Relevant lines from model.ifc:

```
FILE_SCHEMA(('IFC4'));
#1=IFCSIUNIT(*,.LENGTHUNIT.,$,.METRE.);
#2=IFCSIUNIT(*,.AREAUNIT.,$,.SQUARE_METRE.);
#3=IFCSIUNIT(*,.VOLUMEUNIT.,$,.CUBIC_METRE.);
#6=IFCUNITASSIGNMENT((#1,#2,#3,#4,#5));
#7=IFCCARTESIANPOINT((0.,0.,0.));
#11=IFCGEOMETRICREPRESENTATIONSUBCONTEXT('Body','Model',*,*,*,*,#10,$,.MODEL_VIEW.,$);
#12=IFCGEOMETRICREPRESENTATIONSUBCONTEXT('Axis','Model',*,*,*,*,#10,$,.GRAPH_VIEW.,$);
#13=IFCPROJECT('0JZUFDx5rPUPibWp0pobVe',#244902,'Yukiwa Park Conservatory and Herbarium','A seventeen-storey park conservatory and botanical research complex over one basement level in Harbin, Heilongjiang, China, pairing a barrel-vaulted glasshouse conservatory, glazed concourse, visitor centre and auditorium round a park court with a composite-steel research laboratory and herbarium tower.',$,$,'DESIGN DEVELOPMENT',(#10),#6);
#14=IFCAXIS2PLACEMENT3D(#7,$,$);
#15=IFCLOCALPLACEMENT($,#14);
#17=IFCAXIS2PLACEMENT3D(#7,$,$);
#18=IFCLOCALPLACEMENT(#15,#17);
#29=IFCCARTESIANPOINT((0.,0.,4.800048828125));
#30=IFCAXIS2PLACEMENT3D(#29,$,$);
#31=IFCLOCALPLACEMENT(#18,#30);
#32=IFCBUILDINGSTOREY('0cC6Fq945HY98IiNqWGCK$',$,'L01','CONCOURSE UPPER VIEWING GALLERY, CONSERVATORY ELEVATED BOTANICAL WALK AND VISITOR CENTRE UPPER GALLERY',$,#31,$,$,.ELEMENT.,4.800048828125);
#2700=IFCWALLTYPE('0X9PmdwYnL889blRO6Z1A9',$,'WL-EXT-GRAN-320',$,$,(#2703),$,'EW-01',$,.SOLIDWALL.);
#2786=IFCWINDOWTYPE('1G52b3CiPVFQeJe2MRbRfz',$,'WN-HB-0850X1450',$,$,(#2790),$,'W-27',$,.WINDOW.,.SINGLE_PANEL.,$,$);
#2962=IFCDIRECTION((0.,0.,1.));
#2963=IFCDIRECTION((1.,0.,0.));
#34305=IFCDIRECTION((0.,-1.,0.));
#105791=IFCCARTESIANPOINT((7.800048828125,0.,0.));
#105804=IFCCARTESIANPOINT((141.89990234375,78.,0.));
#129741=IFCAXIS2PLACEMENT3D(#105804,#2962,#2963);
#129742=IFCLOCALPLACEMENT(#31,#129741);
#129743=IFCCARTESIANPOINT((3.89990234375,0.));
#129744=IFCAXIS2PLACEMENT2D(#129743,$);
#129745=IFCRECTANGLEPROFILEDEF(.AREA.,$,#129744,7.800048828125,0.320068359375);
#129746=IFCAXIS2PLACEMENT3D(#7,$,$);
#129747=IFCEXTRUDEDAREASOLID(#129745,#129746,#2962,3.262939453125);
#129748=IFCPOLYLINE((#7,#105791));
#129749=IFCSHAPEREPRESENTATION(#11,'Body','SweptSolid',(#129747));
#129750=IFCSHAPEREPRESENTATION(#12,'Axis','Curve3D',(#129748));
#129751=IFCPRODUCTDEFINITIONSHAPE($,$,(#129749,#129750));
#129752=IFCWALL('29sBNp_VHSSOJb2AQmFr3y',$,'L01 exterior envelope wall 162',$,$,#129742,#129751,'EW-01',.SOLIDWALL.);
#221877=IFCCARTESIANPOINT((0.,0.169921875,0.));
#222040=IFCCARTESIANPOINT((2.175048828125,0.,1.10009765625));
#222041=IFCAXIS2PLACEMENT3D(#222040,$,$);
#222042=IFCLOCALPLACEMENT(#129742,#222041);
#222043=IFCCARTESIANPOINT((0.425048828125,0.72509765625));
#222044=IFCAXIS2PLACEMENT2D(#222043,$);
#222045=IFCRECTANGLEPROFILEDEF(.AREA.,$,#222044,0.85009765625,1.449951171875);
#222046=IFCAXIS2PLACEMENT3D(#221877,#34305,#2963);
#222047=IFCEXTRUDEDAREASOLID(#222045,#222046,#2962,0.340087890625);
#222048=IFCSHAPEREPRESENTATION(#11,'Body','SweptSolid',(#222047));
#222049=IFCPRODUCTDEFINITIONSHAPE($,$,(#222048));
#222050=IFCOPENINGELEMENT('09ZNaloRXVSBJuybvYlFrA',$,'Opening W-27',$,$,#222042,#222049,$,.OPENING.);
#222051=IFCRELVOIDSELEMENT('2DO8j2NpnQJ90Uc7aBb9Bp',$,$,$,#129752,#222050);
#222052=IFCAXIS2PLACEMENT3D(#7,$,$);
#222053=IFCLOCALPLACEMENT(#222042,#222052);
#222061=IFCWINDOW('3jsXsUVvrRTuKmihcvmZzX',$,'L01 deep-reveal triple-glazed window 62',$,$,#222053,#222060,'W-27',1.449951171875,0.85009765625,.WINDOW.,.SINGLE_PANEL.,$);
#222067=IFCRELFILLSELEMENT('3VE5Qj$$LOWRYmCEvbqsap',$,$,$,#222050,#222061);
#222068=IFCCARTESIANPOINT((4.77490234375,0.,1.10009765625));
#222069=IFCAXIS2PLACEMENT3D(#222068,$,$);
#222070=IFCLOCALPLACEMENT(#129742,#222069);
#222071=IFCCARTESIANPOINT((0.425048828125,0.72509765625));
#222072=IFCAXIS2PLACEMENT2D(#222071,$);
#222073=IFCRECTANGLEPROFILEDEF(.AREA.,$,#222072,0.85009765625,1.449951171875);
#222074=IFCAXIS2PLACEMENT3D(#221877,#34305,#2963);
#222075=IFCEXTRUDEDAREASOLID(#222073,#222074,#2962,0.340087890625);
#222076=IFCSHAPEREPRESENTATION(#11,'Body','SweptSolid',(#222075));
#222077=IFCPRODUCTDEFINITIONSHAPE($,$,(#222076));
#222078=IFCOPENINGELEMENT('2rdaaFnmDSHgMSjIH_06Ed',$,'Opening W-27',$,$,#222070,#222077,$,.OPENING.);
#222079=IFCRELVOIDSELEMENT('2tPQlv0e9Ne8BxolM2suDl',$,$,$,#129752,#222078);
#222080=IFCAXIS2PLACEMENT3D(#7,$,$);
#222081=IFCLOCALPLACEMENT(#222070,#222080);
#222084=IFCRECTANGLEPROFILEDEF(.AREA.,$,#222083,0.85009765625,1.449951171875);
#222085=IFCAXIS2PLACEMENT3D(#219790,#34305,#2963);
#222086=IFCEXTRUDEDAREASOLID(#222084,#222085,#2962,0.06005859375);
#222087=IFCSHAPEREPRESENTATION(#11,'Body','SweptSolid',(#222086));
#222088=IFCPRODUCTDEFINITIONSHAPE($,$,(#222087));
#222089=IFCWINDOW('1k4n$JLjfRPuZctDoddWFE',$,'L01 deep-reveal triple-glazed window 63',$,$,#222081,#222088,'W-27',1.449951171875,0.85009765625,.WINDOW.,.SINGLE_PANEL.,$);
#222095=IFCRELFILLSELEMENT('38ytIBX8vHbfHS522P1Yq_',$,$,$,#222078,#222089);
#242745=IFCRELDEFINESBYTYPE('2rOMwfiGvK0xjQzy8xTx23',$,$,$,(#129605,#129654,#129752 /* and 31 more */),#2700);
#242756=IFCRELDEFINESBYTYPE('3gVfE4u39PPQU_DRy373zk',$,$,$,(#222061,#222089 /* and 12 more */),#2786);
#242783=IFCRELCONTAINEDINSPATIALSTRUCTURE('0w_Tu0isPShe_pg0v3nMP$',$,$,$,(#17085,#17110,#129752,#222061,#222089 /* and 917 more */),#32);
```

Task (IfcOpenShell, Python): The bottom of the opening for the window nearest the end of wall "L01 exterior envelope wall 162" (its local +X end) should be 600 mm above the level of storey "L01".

```python
import numpy as np
import ifcopenshell
import ifcopenshell.api.geometry
import ifcopenshell.geom
import ifcopenshell.util.element
import ifcopenshell.util.placement
import ifcopenshell.util.shape
import ifcopenshell.util.unit

model = ifcopenshell.open("model.ifc")
unit_scale = ifcopenshell.util.unit.calculate_unit_scale(model)

window = model.by_id(222089)
opening = window.FillsVoids[0].RelatingOpeningElement
storey = ifcopenshell.util.element.get_container(window, ifc_class="IfcBuildingStorey")
level = ifcopenshell.util.placement.get_local_placement(storey.ObjectPlacement)[2, 3]

# The opening's origin need not be at the sill, so measure its lowest point.
shape = ifcopenshell.geom.create_shape(ifcopenshell.geom.settings(), opening)
bottom = ifcopenshell.util.shape.get_shape_bottom_elevation(shape, shape.geometry) / unit_scale
dz = level + 0.6 / unit_scale - bottom

shift = np.array([0.0, 0.0, dz])
# The window is placed relative to its opening, so it follows when the opening moves.
matrix = ifcopenshell.util.placement.get_local_placement(opening.ObjectPlacement)
matrix[:3, 3] += shift
ifcopenshell.api.geometry.edit_object_placement(
    model, product=opening, matrix=matrix, is_si=False, should_transform_children=True
)

print(f"moved by {dz * unit_scale:+.3f} m")

model.write("model-out.ifc")
```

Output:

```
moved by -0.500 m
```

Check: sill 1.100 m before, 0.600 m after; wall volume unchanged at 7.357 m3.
